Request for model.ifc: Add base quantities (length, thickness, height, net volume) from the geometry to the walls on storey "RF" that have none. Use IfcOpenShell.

First a look at what the model holds.

```python
import ifcopenshell
import ifcopenshell.util.element
import ifcopenshell.util.unit

model = ifcopenshell.open("model.ifc")
print(model.schema)
for unit_type in ("LENGTHUNIT", "AREAUNIT", "VOLUMEUNIT"):
    print(unit_type, ifcopenshell.util.unit.calculate_unit_scale(model, unit_type))
storey = next(s for s in model.by_type("IfcBuildingStorey") if s.Name == "RF")
walls = [e for e in ifcopenshell.util.element.get_decomposition(storey) if e.is_a("IfcWall")]
for e in sorted(walls, key=lambda e: e.id()):
    print(e.id(), e.is_a(), e.Name, list(ifcopenshell.util.element.get_psets(e, qtos_only=True)), sep=" | ")
```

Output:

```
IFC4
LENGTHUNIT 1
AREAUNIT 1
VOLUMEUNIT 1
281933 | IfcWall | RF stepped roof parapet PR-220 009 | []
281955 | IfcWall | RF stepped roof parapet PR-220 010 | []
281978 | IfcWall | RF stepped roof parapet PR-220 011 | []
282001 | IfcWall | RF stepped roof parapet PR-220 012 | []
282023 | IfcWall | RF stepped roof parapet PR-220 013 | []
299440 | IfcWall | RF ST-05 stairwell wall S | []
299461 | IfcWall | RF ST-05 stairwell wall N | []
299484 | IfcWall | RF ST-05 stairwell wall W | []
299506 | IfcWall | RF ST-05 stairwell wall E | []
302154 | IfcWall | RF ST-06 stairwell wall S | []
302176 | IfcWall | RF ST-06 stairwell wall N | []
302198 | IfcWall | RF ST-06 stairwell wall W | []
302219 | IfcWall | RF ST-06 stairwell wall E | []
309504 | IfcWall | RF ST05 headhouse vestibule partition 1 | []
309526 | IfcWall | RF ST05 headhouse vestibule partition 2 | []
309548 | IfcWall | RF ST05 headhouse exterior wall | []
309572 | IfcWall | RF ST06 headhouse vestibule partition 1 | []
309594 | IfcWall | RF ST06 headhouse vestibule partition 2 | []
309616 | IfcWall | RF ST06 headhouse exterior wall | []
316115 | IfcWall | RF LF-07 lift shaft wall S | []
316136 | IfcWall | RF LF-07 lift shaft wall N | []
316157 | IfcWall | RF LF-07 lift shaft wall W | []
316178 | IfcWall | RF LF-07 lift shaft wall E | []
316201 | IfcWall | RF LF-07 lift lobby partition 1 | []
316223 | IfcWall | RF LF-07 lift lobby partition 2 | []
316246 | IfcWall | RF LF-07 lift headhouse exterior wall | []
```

```python
import ifcopenshell
import ifcopenshell.api.pset
import ifcopenshell.geom
import ifcopenshell.util.element
import ifcopenshell.util.shape
import ifcopenshell.util.unit

model = ifcopenshell.open("model.ifc")
unit_scale = ifcopenshell.util.unit.calculate_unit_scale(model)
volume_scale = ifcopenshell.util.unit.calculate_unit_scale(model, "VOLUMEUNIT")
settings = ifcopenshell.geom.settings()

storey = next(s for s in model.by_type("IfcBuildingStorey") if s.Name == "RF")
walls = [e for e in ifcopenshell.util.element.get_decomposition(storey) if e.is_a("IfcWall")]

for e in sorted(walls, key=lambda e: e.id()):
    if ifcopenshell.util.element.get_psets(e, qtos_only=True, should_inherit=False):
        continue
    # Geometry comes back in metres, in the element's own axes.
    shape = ifcopenshell.geom.create_shape(settings, e)
    values = {
        "Length": ifcopenshell.util.shape.get_x(shape.geometry) / unit_scale,
        "Width": ifcopenshell.util.shape.get_y(shape.geometry) / unit_scale,
        "Height": ifcopenshell.util.shape.get_z(shape.geometry) / unit_scale,
        "NetVolume": ifcopenshell.util.shape.get_volume(shape.geometry) / volume_scale,
    }
    qto = ifcopenshell.api.pset.add_qto(model, product=e, name="Qto_WallBaseQuantities")
    ifcopenshell.api.pset.edit_qto(model, qto=qto, properties=values)
    print(e.id(), {k: round(v, 3) for k, v in values.items()})

model.write("model_updated.ifc")
```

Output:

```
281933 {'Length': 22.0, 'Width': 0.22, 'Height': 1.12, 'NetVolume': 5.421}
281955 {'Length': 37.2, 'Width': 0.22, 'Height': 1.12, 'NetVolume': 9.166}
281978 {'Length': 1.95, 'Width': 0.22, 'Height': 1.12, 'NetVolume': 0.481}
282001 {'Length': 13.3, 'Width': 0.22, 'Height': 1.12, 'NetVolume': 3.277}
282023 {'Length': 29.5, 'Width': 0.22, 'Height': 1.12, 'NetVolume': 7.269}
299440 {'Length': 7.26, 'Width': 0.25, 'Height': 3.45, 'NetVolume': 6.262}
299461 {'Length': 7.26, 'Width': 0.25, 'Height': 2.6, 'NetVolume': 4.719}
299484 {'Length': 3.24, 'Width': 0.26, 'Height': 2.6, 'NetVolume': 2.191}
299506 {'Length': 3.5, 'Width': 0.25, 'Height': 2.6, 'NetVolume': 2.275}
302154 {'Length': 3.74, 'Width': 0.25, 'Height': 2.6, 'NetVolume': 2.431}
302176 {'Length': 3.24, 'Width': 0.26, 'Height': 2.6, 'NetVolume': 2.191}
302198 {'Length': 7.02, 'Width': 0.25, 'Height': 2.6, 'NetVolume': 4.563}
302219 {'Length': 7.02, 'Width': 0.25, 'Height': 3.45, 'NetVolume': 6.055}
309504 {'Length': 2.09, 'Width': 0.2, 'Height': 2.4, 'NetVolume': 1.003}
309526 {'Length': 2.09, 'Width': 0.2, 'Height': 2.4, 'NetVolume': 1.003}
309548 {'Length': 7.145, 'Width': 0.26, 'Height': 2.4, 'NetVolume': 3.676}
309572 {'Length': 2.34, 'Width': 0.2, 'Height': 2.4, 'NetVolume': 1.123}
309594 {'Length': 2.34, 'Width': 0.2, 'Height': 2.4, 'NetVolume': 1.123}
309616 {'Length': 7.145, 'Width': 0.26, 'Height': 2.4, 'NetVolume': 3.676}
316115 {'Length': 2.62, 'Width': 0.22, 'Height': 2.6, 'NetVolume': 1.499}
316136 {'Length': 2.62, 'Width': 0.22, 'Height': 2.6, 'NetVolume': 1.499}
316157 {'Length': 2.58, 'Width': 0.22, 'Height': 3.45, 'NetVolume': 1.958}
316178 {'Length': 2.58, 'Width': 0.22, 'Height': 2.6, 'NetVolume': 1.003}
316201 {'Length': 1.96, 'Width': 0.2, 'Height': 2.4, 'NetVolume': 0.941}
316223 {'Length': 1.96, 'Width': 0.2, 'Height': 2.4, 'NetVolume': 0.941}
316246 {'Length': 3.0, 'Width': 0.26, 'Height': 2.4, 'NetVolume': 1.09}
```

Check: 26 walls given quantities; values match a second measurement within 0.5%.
